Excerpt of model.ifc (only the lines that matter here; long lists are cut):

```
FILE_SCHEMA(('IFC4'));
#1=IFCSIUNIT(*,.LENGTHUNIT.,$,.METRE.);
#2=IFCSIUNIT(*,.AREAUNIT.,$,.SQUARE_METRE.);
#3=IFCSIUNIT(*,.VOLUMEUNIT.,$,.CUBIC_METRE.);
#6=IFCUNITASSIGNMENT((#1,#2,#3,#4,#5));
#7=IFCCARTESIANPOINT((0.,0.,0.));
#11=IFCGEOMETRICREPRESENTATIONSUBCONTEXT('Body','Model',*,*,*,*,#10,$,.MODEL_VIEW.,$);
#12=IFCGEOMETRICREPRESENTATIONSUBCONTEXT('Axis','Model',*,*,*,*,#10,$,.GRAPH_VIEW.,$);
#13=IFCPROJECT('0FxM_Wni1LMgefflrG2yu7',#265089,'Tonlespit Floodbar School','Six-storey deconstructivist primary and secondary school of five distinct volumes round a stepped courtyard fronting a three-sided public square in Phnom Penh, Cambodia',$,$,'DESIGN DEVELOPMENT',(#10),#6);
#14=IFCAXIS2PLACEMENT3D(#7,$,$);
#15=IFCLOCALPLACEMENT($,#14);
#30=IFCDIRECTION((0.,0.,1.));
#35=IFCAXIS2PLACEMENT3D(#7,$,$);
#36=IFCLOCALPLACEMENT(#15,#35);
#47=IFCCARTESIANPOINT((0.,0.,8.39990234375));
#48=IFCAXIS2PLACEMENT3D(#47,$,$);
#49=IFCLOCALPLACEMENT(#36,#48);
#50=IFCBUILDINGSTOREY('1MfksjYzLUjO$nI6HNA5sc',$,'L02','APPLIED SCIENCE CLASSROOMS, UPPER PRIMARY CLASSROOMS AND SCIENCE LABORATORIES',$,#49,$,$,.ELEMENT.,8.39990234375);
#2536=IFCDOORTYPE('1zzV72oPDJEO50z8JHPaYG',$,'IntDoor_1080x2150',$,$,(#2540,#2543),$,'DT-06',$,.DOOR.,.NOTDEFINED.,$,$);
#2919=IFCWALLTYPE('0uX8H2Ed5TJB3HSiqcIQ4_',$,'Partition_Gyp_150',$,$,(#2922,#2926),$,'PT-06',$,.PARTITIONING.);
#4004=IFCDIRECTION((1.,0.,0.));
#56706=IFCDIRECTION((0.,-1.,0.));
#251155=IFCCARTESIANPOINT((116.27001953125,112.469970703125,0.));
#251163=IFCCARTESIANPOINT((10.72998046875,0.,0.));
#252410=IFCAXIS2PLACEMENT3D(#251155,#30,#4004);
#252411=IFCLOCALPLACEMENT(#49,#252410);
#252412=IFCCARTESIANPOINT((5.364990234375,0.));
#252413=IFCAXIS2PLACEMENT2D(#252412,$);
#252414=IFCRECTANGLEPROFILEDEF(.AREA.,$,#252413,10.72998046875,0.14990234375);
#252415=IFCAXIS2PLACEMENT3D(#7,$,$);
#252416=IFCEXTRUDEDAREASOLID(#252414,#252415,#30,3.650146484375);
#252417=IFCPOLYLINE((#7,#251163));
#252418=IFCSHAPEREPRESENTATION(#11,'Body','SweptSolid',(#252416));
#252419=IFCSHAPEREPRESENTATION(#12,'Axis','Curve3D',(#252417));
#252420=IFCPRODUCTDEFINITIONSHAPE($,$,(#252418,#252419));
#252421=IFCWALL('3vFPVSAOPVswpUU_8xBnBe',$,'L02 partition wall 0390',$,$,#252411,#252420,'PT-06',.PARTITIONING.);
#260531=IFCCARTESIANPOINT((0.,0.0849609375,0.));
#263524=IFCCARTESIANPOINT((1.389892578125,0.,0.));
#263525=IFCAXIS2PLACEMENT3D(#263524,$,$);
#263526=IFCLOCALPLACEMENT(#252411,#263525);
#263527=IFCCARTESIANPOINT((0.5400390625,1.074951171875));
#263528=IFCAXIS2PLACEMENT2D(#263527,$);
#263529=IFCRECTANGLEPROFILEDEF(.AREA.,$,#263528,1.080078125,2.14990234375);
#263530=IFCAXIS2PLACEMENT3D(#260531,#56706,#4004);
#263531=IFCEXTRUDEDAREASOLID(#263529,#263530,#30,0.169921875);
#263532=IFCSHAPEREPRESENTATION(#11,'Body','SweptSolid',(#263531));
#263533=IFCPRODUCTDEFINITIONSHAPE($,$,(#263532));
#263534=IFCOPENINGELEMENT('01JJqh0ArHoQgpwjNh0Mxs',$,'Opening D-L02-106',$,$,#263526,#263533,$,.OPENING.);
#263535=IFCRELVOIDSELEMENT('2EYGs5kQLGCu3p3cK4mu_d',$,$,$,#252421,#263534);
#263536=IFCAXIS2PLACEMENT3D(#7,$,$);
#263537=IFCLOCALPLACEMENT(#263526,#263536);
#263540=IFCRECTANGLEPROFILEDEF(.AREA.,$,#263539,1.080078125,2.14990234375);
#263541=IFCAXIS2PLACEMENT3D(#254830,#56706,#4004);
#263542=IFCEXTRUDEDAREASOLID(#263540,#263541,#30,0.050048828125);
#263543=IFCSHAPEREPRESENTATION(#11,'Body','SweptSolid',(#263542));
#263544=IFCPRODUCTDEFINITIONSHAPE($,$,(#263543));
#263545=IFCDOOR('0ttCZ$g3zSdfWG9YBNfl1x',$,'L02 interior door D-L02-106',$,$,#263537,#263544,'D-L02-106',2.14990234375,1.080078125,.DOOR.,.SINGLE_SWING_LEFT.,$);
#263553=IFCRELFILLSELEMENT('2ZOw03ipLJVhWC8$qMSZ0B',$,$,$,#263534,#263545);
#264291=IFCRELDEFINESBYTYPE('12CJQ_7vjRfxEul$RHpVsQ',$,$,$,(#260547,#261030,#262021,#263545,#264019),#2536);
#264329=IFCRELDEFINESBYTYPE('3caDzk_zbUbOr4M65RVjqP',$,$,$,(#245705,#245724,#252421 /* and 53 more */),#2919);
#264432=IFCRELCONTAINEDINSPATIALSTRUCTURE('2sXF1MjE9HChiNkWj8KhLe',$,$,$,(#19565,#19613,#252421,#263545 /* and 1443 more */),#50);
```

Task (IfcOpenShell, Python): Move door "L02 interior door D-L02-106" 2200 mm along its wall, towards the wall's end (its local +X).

```python
import ifcopenshell
import ifcopenshell.api.geometry
import ifcopenshell.util.placement

model = ifcopenshell.open("model.ifc")

door = model.by_id(263545)
opening = door.FillsVoids[0].RelatingOpeningElement
wall = opening.VoidsElements[0].RelatingBuildingElement

wall_matrix = ifcopenshell.util.placement.get_local_placement(wall.ObjectPlacement)
shift = wall_matrix[:3, 0] * 2.2
before = ifcopenshell.util.placement.get_local_placement(door.ObjectPlacement)[:3, 3].copy()

# The door is placed relative to its opening, so it follows when the opening moves.
matrix = ifcopenshell.util.placement.get_local_placement(opening.ObjectPlacement)
matrix[:3, 3] += shift
ifcopenshell.api.geometry.edit_object_placement(
    model, product=opening, matrix=matrix, is_si=False, should_transform_children=True
)

after = ifcopenshell.util.placement.get_local_placement(door.ObjectPlacement)[:3, 3]
print("door moved by", (after - before).round(3) + 0.0)

model.write("model-out.ifc")
```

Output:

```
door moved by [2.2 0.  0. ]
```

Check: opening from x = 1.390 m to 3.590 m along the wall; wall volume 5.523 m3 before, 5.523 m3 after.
